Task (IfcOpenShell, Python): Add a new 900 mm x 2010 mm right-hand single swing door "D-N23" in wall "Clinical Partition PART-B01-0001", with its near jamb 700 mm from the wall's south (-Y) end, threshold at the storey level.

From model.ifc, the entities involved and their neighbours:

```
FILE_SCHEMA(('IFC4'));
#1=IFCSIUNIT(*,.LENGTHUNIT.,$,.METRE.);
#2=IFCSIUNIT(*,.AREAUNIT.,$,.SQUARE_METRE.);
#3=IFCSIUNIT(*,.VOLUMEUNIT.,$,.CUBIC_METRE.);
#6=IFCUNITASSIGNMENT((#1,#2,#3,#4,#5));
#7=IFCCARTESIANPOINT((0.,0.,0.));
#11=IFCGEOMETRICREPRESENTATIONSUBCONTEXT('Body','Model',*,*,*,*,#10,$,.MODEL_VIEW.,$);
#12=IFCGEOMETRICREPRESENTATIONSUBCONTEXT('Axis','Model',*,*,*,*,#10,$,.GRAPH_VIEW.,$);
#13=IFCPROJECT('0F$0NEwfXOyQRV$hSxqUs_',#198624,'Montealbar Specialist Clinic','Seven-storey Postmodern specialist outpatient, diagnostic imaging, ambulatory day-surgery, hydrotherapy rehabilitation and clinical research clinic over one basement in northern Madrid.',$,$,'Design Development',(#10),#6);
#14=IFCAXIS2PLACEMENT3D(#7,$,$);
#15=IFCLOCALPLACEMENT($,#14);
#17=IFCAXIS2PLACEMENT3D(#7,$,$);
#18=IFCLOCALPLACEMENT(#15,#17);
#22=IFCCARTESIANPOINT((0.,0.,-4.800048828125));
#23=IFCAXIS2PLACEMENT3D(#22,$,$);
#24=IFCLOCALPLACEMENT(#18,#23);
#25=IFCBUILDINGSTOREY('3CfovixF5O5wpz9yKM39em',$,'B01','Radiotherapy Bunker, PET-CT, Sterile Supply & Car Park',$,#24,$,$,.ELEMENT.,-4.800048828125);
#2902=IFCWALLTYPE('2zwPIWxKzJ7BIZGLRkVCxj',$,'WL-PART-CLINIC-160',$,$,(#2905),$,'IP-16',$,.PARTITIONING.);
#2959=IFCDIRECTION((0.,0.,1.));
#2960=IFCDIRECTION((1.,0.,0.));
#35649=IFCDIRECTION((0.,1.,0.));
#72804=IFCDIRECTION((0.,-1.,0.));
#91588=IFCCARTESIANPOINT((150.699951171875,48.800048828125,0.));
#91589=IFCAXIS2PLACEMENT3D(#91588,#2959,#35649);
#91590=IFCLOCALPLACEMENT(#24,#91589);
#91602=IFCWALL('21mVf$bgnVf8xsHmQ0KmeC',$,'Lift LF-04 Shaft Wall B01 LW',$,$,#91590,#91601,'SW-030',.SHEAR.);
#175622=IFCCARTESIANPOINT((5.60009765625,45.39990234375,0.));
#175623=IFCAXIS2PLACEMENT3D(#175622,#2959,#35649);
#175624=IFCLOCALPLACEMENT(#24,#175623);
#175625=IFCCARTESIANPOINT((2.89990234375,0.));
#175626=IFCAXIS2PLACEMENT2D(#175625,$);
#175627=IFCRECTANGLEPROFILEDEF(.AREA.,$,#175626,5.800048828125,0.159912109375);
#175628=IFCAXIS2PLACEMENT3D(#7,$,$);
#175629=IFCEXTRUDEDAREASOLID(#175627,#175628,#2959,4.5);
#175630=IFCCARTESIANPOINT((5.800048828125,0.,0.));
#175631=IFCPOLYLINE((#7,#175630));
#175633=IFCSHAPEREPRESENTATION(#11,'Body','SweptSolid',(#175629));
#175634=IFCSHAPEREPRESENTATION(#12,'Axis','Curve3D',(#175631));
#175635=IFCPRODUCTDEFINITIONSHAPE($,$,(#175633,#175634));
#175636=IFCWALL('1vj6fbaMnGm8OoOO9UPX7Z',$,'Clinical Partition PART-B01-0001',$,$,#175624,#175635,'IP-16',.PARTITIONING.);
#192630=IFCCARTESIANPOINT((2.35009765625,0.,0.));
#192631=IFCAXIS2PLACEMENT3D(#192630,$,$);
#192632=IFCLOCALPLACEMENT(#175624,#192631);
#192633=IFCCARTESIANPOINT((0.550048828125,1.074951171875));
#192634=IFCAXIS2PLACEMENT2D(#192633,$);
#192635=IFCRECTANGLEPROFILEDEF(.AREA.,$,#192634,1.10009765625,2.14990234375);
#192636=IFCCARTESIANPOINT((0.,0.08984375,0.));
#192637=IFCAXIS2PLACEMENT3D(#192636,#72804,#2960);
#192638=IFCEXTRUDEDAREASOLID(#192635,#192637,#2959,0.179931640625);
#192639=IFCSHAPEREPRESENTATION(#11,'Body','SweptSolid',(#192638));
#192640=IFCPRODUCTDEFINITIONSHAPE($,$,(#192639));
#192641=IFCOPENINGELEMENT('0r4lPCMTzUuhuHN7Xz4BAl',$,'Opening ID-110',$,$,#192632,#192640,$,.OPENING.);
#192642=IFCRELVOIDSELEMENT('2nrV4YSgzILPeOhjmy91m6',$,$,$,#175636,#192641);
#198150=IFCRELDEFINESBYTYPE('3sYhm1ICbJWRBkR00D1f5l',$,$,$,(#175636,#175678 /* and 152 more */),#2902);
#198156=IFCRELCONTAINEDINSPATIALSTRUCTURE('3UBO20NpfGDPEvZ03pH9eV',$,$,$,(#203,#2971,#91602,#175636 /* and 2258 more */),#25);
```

```python
import numpy as np
import ifcopenshell
import ifcopenshell.api.feature
import ifcopenshell.api.geometry
import ifcopenshell.api.root
import ifcopenshell.api.spatial
import ifcopenshell.geom
import ifcopenshell.util.element
import ifcopenshell.util.placement
import ifcopenshell.util.representation
import ifcopenshell.util.shape
import ifcopenshell.util.unit

model = ifcopenshell.open("model.ifc")
unit_scale = ifcopenshell.util.unit.calculate_unit_scale(model)
settings = ifcopenshell.geom.settings()


def volume(element):
    """Net volume in cubic metres, openings subtracted."""
    shape = ifcopenshell.geom.create_shape(settings, element)
    return ifcopenshell.util.shape.get_volume(shape.geometry)


wall = model.by_guid("1vj6fbaMnGm8OoOO9UPX7Z")
storey = ifcopenshell.util.element.get_container(wall, ifc_class="IfcBuildingStorey")
context = ifcopenshell.util.representation.get_context(model, "Model", "Body", "MODEL_VIEW")
before = volume(wall)

width, height, from_end, sill = 0.9, 2.01, 0.7, 0.0  # metres

# The wall runs along its own X axis, and the end named is its -X end.
wall_shape = ifcopenshell.geom.create_shape(settings, wall)
x, y, z = ifcopenshell.util.shape.get_vertices(wall_shape.geometry).T
start = x.min() + from_end
face, thickness = float(y.min()), float(y.max() - y.min())
wall_matrix = ifcopenshell.util.placement.get_local_placement(wall.ObjectPlacement)
level = ifcopenshell.util.placement.get_local_placement(storey.ObjectPlacement)[2, 3]


def in_wall(x, y):
    """Placement at x, y metres in the wall's axes, at sill height."""
    matrix = wall_matrix.copy()
    matrix[:, 3] = wall_matrix @ np.array([x / unit_scale, y / unit_scale, 0.0, 1.0])
    matrix[2, 3] = level + sill / unit_scale
    return matrix


# Opening: a box that overshoots both wall faces by 50 mm.
opening = ifcopenshell.api.root.create_entity(model, ifc_class="IfcOpeningElement", predefined_type="OPENING")
box = ifcopenshell.api.geometry.add_wall_representation(
    model, context=context, length=width, height=height, thickness=thickness + 0.1
)
ifcopenshell.api.geometry.assign_representation(model, product=opening, representation=box)
ifcopenshell.api.geometry.edit_object_placement(model, product=opening, matrix=in_wall(start, face - 0.05), is_si=False)
ifcopenshell.api.feature.add_feature(model, feature=opening, element=wall)

door = ifcopenshell.api.root.create_entity(model, ifc_class="IfcDoor", name="D-N23", predefined_type="DOOR")
door.OverallWidth, door.OverallHeight = width / unit_scale, height / unit_scale
door.OperationType = "SINGLE_SWING_RIGHT"
body = ifcopenshell.api.geometry.add_door_representation(
    model,
    context=context,
    overall_width=door.OverallWidth,
    overall_height=door.OverallHeight,
    operation_type="SINGLE_SWING_RIGHT",
    lining_properties={"LiningDepth": thickness / unit_scale, "ThresholdDepth": thickness / unit_scale},
)
ifcopenshell.api.geometry.assign_representation(model, product=door, representation=body)
ifcopenshell.api.spatial.assign_container(model, products=[door], relating_structure=storey)
ifcopenshell.api.feature.add_filling(model, opening=opening, element=door)

# The lining spans the wall, so the door starts at the wall face.
ifcopenshell.api.geometry.edit_object_placement(model, product=door, matrix=in_wall(start, face), is_si=False)

after = volume(wall)

print(f"wall volume {before:.3f} -> {after:.3f} m3")

model.write("model_rev.ifc")
```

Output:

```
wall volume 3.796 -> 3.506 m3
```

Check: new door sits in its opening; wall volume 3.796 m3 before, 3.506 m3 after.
